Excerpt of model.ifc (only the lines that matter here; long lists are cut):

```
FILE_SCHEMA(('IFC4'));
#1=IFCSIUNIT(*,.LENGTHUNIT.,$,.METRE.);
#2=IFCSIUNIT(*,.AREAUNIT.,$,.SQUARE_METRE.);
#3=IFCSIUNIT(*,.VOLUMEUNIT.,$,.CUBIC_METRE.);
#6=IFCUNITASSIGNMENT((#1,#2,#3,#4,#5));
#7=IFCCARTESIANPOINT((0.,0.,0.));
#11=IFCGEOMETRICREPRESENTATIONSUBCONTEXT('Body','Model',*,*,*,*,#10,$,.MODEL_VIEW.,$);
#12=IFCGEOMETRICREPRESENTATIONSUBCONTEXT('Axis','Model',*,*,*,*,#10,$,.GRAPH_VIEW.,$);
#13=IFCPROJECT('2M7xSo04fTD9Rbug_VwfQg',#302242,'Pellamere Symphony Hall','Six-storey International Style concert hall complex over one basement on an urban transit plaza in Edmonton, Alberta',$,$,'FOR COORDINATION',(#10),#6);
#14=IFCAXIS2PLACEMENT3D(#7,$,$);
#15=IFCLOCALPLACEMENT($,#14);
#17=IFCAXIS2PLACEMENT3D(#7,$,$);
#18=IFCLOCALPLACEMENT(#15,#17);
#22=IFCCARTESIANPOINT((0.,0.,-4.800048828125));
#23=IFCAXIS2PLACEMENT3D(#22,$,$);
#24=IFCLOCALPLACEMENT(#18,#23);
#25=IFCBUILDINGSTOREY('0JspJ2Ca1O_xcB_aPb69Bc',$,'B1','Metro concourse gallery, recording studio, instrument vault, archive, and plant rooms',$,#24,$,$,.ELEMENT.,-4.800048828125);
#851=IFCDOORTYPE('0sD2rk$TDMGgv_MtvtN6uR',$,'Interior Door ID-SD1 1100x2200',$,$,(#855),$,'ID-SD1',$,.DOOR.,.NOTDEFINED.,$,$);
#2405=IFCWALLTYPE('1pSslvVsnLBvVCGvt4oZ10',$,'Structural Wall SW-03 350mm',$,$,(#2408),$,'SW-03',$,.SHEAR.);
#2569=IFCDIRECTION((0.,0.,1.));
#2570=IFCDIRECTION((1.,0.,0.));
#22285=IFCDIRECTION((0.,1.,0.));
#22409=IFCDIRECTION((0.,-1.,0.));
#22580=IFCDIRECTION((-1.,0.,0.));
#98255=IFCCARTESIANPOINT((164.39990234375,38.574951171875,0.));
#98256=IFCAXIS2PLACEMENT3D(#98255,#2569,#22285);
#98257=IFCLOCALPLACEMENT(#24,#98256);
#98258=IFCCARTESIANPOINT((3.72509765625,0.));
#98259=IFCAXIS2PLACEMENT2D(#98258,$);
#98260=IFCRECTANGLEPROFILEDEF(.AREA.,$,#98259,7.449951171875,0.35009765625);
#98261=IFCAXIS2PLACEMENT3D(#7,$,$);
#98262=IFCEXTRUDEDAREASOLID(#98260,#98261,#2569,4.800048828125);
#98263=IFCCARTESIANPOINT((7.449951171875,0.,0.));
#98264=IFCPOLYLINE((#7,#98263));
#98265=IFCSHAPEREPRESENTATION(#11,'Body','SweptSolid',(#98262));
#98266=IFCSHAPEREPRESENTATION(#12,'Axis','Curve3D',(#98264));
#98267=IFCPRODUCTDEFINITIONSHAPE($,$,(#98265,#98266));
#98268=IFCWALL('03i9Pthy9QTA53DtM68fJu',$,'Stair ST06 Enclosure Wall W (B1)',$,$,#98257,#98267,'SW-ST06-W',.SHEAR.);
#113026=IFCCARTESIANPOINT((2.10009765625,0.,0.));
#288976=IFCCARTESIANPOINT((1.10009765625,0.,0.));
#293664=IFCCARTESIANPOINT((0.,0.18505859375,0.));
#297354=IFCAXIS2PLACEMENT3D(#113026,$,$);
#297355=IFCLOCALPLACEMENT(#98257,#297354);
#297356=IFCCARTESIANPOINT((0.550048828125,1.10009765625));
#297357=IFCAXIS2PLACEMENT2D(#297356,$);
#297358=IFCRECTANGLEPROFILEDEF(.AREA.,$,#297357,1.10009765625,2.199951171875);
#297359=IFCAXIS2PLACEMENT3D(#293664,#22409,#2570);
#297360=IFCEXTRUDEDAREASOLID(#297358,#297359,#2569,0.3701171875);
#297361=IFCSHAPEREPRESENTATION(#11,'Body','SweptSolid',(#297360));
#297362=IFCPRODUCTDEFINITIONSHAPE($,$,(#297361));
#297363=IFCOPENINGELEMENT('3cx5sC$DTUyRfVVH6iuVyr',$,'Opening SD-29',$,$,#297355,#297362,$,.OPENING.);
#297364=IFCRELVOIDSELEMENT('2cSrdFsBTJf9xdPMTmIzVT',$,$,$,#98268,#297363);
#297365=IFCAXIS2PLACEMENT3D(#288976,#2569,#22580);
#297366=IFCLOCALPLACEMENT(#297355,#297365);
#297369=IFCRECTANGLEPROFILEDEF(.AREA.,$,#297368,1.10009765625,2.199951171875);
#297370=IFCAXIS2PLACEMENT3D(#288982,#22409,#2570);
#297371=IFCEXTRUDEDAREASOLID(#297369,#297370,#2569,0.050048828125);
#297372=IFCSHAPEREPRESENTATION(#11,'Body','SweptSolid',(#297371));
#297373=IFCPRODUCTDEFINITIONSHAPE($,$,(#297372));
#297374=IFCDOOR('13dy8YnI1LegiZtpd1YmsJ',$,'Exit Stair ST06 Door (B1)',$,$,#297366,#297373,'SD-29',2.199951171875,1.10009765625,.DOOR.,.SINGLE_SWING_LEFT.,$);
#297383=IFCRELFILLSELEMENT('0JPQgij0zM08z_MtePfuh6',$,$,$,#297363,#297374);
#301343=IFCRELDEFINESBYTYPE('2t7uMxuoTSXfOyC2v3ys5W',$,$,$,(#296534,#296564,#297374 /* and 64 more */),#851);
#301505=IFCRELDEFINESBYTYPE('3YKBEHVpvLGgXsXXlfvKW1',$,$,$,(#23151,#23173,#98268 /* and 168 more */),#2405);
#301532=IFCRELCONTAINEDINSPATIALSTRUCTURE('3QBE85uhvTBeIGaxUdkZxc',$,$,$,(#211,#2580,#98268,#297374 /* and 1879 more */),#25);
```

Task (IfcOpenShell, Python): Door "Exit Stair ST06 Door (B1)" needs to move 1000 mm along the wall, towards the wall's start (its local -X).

```python
import ifcopenshell
import ifcopenshell.api.geometry
import ifcopenshell.util.placement

model = ifcopenshell.open("model.ifc")

door = model.by_guid("13dy8YnI1LegiZtpd1YmsJ")
opening = door.FillsVoids[0].RelatingOpeningElement
wall = opening.VoidsElements[0].RelatingBuildingElement

wall_matrix = ifcopenshell.util.placement.get_local_placement(wall.ObjectPlacement)
shift = wall_matrix[:3, 0] * -1.0
before = ifcopenshell.util.placement.get_local_placement(door.ObjectPlacement)[:3, 3].copy()

# The door is placed relative to its opening, so it follows when the opening moves.
matrix = ifcopenshell.util.placement.get_local_placement(opening.ObjectPlacement)
matrix[:3, 3] += shift
ifcopenshell.api.geometry.edit_object_placement(
    model, product=opening, matrix=matrix, is_si=False, should_transform_children=True
)

after = ifcopenshell.util.placement.get_local_placement(door.ObjectPlacement)[:3, 3]
print("door moved by", (after - before).round(3) + 0.0)

model.write("model_updated.ifc")
```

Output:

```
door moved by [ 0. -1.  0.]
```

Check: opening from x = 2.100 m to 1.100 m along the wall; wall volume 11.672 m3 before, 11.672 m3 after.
